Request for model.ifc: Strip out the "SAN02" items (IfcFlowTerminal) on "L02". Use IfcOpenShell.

First a look at what the model holds.

```python
import ifcopenshell
import ifcopenshell.util.element

model = ifcopenshell.open("model.ifc")
print(model.schema)
storey = next(s for s in model.by_type("IfcBuildingStorey") if s.Name == "L02")
terminals = [e for e in ifcopenshell.util.element.get_decomposition(storey) if e.is_a("IfcFlowTerminal")]
seen = {}
for e in terminals:
    element_type = ifcopenshell.util.element.get_type(e)
    name = element_type.Name if element_type not in (None, e) else None
    seen[name] = seen.get(name, 0) + 1
for name, count in sorted(seen.items(), key=str):
    print(count, "x", name)
```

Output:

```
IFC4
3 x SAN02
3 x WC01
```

```python
import ifcopenshell
import ifcopenshell.api.root
import ifcopenshell.util.element

model = ifcopenshell.open("model.ifc")

storey = next(s for s in model.by_type("IfcBuildingStorey") if s.Name == "L02")
terminals = [e for e in ifcopenshell.util.element.get_decomposition(storey) if e.is_a("IfcFlowTerminal")]
targets = [e for e in terminals if (t := ifcopenshell.util.element.get_type(e)) not in (None, e) and t.Name == "SAN02"]

for e in targets:
    ifcopenshell.api.root.remove_product(model, product=e)
print(len(targets), "removed")

model.write("model-out.ifc")
```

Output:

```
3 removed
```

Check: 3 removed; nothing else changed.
